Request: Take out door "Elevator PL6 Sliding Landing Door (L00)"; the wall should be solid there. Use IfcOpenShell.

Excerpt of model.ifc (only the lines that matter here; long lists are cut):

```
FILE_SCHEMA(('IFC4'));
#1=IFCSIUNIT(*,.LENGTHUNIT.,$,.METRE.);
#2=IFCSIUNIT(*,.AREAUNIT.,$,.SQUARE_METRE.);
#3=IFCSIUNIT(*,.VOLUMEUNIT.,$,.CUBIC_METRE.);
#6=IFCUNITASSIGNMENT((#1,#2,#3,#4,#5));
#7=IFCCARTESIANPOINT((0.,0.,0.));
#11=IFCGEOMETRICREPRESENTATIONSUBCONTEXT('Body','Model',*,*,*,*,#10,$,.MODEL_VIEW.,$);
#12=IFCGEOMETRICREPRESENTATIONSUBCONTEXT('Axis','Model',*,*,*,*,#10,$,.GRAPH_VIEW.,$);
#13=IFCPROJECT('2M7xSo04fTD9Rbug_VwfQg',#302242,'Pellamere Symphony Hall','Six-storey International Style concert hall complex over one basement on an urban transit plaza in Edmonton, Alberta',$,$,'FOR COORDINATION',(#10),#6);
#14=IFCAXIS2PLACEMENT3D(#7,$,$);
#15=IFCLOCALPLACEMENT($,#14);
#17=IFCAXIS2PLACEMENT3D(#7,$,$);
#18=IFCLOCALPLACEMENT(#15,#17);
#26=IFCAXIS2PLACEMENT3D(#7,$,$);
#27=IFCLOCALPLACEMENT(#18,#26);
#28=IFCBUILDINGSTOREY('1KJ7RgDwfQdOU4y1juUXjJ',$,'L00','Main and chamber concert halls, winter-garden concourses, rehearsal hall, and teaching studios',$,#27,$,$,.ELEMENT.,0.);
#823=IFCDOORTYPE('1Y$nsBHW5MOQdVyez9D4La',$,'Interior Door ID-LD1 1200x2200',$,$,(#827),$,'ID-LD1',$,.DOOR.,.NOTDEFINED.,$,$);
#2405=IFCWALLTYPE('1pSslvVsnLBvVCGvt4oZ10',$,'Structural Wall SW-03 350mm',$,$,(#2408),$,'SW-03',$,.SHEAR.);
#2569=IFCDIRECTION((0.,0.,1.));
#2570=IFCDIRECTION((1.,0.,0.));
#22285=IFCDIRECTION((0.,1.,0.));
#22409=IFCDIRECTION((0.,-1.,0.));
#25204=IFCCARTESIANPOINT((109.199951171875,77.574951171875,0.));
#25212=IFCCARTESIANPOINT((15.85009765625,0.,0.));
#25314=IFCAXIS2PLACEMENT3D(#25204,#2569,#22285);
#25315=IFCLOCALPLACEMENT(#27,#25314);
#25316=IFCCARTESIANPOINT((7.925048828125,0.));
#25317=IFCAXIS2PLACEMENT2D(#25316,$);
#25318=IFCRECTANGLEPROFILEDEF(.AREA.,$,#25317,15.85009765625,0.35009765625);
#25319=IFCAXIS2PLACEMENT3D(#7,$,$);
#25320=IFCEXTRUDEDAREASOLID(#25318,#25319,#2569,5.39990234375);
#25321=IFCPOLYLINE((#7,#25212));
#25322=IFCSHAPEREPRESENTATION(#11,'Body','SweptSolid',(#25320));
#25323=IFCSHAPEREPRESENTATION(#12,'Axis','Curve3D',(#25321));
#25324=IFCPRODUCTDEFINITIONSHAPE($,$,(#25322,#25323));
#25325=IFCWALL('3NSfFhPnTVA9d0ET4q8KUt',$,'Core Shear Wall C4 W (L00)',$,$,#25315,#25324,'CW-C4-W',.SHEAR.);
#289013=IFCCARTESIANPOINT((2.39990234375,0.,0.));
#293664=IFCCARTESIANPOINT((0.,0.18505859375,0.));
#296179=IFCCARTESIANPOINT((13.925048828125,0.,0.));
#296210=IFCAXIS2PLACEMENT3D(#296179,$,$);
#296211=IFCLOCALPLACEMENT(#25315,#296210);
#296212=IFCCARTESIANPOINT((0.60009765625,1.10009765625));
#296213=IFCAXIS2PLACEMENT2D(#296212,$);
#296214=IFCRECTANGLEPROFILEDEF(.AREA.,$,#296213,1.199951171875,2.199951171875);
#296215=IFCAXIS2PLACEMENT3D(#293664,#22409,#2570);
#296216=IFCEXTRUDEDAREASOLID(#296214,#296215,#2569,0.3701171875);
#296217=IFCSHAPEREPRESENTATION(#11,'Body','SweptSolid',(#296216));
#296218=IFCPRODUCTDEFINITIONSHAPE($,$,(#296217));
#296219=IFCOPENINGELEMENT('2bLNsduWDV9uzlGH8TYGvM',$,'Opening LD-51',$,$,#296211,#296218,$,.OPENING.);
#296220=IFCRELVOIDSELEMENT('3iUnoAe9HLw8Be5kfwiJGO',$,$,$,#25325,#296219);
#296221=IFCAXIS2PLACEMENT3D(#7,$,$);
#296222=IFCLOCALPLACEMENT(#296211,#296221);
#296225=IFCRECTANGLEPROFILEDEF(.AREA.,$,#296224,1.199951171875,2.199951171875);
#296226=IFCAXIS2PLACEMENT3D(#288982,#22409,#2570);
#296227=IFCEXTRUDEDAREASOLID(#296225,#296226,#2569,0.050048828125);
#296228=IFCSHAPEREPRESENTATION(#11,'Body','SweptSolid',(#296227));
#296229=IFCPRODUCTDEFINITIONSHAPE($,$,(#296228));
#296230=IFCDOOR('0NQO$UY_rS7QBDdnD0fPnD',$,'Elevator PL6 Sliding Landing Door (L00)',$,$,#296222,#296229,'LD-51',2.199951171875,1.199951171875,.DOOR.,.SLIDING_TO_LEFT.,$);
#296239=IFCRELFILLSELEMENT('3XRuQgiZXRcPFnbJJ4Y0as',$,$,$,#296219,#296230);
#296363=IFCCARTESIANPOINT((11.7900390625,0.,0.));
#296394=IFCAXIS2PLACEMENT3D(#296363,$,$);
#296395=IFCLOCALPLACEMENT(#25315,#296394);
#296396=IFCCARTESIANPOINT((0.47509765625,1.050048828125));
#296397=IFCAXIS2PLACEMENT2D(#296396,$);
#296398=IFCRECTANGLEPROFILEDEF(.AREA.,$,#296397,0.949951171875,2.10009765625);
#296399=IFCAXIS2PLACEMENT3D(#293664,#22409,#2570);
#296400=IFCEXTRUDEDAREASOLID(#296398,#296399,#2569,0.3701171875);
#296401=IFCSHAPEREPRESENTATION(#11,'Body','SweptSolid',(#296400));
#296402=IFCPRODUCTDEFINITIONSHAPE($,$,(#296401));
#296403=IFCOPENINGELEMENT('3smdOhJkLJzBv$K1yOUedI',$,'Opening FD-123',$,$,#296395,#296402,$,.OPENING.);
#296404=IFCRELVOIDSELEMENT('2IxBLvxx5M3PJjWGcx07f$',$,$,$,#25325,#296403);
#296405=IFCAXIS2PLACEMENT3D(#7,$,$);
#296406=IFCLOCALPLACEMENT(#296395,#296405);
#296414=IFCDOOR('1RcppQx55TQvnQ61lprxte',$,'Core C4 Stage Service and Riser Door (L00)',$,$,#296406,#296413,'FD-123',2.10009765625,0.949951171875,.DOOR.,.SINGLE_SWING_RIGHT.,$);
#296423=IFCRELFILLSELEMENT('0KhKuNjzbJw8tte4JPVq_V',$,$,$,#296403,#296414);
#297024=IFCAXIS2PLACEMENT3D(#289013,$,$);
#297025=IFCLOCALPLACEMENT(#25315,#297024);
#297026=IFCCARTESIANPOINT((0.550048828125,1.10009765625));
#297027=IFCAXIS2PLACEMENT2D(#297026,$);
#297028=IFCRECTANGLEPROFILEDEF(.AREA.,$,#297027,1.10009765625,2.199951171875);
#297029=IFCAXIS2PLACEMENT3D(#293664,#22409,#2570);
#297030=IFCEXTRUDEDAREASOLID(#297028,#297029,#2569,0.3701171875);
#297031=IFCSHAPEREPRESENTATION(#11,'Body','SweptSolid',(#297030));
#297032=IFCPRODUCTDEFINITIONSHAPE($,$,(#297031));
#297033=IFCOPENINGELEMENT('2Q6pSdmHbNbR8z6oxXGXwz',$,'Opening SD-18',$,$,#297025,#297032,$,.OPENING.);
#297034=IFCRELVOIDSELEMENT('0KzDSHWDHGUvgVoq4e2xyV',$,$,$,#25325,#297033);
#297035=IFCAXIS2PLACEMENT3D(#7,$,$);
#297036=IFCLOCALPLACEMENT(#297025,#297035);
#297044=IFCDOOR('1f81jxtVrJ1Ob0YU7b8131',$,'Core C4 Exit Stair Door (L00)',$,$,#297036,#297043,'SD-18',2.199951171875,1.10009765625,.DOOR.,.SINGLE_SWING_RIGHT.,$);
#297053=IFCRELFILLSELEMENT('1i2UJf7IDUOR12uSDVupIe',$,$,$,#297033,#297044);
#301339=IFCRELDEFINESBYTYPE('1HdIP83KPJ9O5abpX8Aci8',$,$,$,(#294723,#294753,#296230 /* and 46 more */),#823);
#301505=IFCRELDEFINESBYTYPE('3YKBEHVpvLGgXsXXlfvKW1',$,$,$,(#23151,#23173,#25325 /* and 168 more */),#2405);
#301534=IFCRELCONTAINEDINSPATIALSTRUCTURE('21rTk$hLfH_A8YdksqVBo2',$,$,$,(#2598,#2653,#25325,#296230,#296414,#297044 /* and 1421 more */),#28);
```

```python
import ifcopenshell
import ifcopenshell.api.feature
import ifcopenshell.api.root
import ifcopenshell.geom
import ifcopenshell.util.shape

model = ifcopenshell.open("model.ifc")
settings = ifcopenshell.geom.settings()


def volume(element):
    """Net volume in cubic metres, openings subtracted."""
    shape = ifcopenshell.geom.create_shape(settings, element)
    return ifcopenshell.util.shape.get_volume(shape.geometry)


door = model.by_guid("0NQO$UY_rS7QBDdnD0fPnD")
opening = door.FillsVoids[0].RelatingOpeningElement
wall = opening.VoidsElements[0].RelatingBuildingElement
before = volume(wall)

ifcopenshell.api.root.remove_product(model, product=door)
ifcopenshell.api.feature.remove_feature(model, feature=opening)

after = volume(wall)

print(f"wall volume {before:.3f} -> {after:.3f} m3")

model.write("model_edited.ifc")
```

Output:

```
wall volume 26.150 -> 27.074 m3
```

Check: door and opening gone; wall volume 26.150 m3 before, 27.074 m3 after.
